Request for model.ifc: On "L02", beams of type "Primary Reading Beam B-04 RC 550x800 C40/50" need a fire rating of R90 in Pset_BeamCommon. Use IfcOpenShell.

First a look at what the model holds.

```python
import ifcopenshell
import ifcopenshell.util.element

model = ifcopenshell.open("model.ifc")
print(model.schema)
storey = next(s for s in model.by_type("IfcBuildingStorey") if s.Name == "L02")
beams = [e for e in ifcopenshell.util.element.get_decomposition(storey) if e.is_a("IfcBeam")]
seen = {}
for e in beams:
    element_type = ifcopenshell.util.element.get_type(e)
    key = (element_type.Name if element_type != e and element_type else None, ifcopenshell.util.element.get_pset(e, "Pset_BeamCommon", "FireRating"))
    seen[key] = seen.get(key, 0) + 1
for (name, value), count in sorted(seen.items(), key=str):
    print(count, "x", name, "|", value)
```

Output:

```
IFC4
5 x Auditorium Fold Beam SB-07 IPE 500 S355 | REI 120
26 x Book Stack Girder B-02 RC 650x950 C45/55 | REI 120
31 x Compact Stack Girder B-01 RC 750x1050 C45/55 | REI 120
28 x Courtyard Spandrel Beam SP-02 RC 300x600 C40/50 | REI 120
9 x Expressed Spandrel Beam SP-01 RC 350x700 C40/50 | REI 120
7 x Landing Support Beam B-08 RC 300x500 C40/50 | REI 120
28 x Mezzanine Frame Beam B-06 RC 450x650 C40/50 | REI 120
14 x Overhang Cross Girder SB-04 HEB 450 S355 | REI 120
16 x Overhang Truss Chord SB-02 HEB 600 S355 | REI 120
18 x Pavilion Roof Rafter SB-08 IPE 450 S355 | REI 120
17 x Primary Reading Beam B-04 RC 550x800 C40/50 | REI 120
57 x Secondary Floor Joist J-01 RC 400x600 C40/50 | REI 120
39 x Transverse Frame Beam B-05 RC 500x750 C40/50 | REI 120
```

```python
import ifcopenshell
import ifcopenshell.api.pset
import ifcopenshell.util.element

model = ifcopenshell.open("model.ifc")

storey = next(s for s in model.by_type("IfcBuildingStorey") if s.Name == "L02")
beams = [e for e in ifcopenshell.util.element.get_decomposition(storey) if e.is_a("IfcBeam")]

count = 0
for e in beams:
    element_type = ifcopenshell.util.element.get_type(e)
    if element_type in (None, e) or element_type.Name != "Primary Reading Beam B-04 RC 550x800 C40/50":
        continue
    # add_pset returns the element's existing set when there is one.
    pset = ifcopenshell.api.pset.add_pset(model, product=e, name="Pset_BeamCommon")
    ifcopenshell.api.pset.edit_pset(model, pset=pset, properties={"FireRating": "R90"})
    count += 1

print(count, "beams updated")

model.write("model_rev.ifc")
```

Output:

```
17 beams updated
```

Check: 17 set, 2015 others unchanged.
